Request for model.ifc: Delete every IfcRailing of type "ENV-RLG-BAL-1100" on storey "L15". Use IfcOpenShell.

First a look at what the model holds.

```python
import ifcopenshell
import ifcopenshell.util.element

model = ifcopenshell.open("model.ifc")
print(model.schema)
storey = next(s for s in model.by_type("IfcBuildingStorey") if s.Name == "L15")
railings = [e for e in ifcopenshell.util.element.get_decomposition(storey) if e.is_a("IfcRailing")]
seen = {}
for e in railings:
    element_type = ifcopenshell.util.element.get_type(e)
    name = element_type.Name if element_type not in (None, e) else None
    seen[name] = seen.get(name, 0) + 1
for name, count in sorted(seen.items(), key=str):
    print(count, "x", name)
```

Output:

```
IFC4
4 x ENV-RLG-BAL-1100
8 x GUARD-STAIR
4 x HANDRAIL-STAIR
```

```python
import ifcopenshell
import ifcopenshell.api.root
import ifcopenshell.util.element

model = ifcopenshell.open("model.ifc")

storey = next(s for s in model.by_type("IfcBuildingStorey") if s.Name == "L15")
railings = [e for e in ifcopenshell.util.element.get_decomposition(storey) if e.is_a("IfcRailing")]
targets = [e for e in railings if (t := ifcopenshell.util.element.get_type(e)) not in (None, e) and t.Name == "ENV-RLG-BAL-1100"]

for e in targets:
    ifcopenshell.api.root.remove_product(model, product=e)
print(len(targets), "removed")

model.write("model-out.ifc")
```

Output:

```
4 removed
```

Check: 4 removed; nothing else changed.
